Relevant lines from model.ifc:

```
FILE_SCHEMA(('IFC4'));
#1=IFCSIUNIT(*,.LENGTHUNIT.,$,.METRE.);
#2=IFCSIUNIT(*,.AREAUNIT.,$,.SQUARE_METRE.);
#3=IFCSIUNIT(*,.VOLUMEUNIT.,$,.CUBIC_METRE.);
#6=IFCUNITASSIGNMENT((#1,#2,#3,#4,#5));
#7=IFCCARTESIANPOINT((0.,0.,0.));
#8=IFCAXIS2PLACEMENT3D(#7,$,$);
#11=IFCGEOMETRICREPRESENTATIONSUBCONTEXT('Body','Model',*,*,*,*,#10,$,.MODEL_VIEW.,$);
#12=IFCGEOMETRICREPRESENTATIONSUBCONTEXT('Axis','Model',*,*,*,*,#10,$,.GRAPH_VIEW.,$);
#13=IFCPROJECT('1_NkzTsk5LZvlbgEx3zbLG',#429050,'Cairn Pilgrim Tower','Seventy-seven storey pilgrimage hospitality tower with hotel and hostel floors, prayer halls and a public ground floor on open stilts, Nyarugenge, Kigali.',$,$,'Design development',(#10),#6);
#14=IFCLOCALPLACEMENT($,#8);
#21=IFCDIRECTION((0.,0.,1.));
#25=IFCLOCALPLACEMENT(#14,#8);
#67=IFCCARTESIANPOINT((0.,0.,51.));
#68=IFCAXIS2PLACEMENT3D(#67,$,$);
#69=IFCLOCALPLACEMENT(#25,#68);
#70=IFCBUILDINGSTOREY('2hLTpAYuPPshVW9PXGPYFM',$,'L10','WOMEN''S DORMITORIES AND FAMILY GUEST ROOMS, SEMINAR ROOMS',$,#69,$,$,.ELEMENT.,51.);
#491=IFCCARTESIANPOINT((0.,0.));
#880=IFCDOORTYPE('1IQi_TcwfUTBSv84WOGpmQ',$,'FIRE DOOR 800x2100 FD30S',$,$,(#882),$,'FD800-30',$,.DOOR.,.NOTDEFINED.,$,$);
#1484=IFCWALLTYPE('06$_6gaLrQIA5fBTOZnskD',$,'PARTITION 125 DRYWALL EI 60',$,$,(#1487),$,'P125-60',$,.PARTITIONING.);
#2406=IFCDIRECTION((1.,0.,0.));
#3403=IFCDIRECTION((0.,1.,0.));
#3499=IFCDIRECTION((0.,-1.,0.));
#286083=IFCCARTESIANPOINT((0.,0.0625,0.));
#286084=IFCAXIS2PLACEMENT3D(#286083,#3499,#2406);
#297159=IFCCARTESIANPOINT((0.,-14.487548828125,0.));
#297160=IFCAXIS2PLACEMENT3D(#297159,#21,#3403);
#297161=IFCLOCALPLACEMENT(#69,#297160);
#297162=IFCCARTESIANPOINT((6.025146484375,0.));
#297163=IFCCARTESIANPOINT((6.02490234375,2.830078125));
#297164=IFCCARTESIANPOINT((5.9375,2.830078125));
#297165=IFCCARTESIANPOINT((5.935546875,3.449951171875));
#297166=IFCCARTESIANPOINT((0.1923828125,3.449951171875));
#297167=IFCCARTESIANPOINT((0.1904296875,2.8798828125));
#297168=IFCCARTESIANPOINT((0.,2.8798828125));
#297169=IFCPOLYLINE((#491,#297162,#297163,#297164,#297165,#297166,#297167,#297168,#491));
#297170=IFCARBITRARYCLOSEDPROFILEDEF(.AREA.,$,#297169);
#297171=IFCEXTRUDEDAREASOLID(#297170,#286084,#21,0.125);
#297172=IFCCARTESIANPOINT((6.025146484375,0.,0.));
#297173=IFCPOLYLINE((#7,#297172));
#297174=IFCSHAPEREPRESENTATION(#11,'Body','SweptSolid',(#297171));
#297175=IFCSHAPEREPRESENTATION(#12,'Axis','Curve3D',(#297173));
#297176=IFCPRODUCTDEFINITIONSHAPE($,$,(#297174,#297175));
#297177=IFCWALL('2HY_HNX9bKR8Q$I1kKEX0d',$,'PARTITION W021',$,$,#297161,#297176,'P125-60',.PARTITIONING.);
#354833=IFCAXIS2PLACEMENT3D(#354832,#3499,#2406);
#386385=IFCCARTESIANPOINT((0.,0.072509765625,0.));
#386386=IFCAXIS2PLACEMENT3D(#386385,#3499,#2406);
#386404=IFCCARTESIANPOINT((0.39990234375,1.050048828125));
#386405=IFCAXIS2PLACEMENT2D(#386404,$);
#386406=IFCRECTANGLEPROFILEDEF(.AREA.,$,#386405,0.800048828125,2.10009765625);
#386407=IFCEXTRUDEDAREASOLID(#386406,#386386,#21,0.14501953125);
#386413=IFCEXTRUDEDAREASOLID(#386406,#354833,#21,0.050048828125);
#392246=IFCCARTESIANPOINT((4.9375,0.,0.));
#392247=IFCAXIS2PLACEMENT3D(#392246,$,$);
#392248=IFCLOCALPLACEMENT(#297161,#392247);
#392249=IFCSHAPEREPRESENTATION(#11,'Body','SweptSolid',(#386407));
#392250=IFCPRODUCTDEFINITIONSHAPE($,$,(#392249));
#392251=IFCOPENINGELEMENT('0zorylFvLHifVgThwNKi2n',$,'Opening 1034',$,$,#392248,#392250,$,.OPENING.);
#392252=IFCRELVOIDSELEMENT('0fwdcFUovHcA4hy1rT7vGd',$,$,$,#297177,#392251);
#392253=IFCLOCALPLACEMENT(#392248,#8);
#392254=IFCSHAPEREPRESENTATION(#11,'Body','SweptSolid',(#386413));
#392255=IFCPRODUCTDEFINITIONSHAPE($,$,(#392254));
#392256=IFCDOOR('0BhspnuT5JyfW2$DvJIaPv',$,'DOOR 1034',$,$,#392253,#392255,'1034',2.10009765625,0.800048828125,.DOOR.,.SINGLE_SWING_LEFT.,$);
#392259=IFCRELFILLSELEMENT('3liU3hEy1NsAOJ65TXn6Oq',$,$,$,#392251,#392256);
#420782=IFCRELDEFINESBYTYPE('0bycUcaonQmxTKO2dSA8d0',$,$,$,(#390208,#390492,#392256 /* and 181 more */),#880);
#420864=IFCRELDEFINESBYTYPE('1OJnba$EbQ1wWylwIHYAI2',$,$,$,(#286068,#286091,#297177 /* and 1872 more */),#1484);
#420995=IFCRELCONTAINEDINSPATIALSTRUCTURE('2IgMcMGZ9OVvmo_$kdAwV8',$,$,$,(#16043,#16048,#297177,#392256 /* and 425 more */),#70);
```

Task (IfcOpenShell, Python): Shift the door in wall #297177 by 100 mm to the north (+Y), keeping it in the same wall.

```python
import ifcopenshell
import ifcopenshell.api.geometry
import ifcopenshell.util.placement
import ifcopenshell.util.unit

model = ifcopenshell.open("model.ifc")
unit_scale = ifcopenshell.util.unit.calculate_unit_scale(model)

door = model.by_guid("0BhspnuT5JyfW2$DvJIaPv")
opening = door.FillsVoids[0].RelatingOpeningElement
wall = opening.VoidsElements[0].RelatingBuildingElement

wall_matrix = ifcopenshell.util.placement.get_local_placement(wall.ObjectPlacement)
shift = wall_matrix[:3, 0] * 0.1 / unit_scale
before = ifcopenshell.util.placement.get_local_placement(door.ObjectPlacement)[:3, 3].copy()

# The door is placed relative to its opening, so it follows when the opening moves.
matrix = ifcopenshell.util.placement.get_local_placement(opening.ObjectPlacement)
matrix[:3, 3] += shift
ifcopenshell.api.geometry.edit_object_placement(
    model, product=opening, matrix=matrix, is_si=False, should_transform_children=True
)

after = ifcopenshell.util.placement.get_local_placement(door.ObjectPlacement)[:3, 3]
print("door moved by", (after - before).round(3) + 0.0)

model.write("model_rev.ifc")
```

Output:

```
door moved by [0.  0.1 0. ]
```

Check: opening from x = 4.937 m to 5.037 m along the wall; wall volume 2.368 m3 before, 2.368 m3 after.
